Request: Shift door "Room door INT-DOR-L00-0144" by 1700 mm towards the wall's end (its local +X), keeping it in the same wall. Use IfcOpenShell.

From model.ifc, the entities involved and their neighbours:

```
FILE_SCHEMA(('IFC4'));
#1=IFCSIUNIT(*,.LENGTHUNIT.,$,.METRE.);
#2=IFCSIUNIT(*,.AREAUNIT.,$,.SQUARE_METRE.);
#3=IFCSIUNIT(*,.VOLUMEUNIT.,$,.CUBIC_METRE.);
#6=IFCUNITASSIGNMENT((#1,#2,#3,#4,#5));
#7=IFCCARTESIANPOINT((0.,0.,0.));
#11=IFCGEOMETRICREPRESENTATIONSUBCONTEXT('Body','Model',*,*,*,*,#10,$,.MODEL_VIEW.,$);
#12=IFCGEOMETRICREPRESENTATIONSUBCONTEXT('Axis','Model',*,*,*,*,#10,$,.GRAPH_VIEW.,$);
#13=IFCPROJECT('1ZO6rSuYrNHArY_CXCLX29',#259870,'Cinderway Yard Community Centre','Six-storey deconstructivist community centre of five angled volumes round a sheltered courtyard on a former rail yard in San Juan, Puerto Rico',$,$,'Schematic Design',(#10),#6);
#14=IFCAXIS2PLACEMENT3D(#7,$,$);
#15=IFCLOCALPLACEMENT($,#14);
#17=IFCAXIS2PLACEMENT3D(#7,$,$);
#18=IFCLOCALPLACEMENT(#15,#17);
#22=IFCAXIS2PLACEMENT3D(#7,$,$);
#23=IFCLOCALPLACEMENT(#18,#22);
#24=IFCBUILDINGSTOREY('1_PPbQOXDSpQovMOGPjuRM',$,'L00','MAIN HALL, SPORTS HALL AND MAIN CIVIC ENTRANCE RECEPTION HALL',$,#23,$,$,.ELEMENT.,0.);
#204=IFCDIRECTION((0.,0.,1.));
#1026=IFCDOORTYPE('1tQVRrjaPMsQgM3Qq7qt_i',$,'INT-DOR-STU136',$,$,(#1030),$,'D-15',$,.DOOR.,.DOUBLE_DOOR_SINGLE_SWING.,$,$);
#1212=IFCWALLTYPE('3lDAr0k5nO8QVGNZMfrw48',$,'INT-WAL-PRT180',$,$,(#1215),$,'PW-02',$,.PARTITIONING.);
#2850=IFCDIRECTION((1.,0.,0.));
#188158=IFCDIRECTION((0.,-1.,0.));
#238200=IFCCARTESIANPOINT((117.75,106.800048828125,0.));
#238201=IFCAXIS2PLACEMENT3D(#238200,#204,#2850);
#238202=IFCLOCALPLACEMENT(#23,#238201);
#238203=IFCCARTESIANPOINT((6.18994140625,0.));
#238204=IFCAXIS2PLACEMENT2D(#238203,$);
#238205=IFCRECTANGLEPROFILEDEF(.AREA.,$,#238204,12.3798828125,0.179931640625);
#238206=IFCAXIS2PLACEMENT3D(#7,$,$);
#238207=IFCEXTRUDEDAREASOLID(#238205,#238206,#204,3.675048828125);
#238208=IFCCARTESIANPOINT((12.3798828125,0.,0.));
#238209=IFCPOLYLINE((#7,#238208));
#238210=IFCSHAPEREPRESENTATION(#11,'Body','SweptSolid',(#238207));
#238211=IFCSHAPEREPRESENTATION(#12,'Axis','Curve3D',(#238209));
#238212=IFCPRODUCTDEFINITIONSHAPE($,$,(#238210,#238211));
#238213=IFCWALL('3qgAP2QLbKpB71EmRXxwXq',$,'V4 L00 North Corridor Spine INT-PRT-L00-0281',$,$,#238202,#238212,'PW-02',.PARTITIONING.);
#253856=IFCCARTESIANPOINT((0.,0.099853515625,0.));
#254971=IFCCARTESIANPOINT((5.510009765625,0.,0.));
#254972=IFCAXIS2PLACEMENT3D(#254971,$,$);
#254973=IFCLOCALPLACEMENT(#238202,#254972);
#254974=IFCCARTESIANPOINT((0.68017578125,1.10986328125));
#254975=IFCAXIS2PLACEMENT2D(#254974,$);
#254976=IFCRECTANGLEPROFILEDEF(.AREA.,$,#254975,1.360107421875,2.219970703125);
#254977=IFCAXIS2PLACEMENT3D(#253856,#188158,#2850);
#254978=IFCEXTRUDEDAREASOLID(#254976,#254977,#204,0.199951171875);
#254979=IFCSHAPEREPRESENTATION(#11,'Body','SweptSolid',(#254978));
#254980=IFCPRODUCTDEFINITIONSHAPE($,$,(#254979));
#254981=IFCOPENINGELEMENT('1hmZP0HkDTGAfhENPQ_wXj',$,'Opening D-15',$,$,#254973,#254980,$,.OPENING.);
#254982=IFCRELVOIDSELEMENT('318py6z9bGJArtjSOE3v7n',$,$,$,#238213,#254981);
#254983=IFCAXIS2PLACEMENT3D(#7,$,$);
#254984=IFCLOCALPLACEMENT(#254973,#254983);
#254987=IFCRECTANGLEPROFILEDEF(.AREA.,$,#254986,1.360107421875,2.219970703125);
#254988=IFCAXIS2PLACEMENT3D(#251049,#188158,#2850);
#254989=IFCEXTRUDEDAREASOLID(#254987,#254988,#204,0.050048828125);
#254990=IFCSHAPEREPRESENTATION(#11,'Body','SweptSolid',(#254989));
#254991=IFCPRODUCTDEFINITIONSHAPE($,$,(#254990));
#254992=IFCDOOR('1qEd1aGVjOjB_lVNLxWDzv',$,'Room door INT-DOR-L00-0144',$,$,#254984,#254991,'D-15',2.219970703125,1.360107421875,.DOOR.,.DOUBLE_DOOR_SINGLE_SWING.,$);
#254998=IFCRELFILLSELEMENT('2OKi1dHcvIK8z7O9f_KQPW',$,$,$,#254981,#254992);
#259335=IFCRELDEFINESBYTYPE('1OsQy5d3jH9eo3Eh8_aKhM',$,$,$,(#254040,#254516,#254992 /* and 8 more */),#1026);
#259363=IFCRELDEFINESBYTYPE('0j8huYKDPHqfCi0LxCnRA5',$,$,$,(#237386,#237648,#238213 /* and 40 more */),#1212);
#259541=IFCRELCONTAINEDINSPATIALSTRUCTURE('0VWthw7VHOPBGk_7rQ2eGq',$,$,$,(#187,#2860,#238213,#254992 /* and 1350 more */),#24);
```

```python
import ifcopenshell
import ifcopenshell.api.geometry
import ifcopenshell.util.placement
import ifcopenshell.util.unit

model = ifcopenshell.open("model.ifc")
unit_scale = ifcopenshell.util.unit.calculate_unit_scale(model)

door = model.by_guid("1qEd1aGVjOjB_lVNLxWDzv")
opening = door.FillsVoids[0].RelatingOpeningElement
wall = opening.VoidsElements[0].RelatingBuildingElement

wall_matrix = ifcopenshell.util.placement.get_local_placement(wall.ObjectPlacement)
shift = wall_matrix[:3, 0] * 1.7 / unit_scale
before = ifcopenshell.util.placement.get_local_placement(door.ObjectPlacement)[:3, 3].copy()

# The door is placed relative to its opening, so it follows when the opening moves.
matrix = ifcopenshell.util.placement.get_local_placement(opening.ObjectPlacement)
matrix[:3, 3] += shift
ifcopenshell.api.geometry.edit_object_placement(
    model, product=opening, matrix=matrix, is_si=False, should_transform_children=True
)

after = ifcopenshell.util.placement.get_local_placement(door.ObjectPlacement)[:3, 3]
print("door moved by", (after - before).round(3) + 0.0)

model.write("model_rev.ifc")
```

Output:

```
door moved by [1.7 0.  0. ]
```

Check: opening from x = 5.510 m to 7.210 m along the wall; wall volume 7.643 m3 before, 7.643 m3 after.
